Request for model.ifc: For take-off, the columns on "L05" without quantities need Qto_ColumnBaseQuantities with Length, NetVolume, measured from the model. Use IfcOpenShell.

First a look at what the model holds.

```python
import ifcopenshell
import ifcopenshell.util.element
import ifcopenshell.util.unit

model = ifcopenshell.open("model.ifc")
print(model.schema)
for unit_type in ("LENGTHUNIT", "AREAUNIT", "VOLUMEUNIT"):
    print(unit_type, ifcopenshell.util.unit.calculate_unit_scale(model, unit_type))
storey = next(s for s in model.by_type("IfcBuildingStorey") if s.Name == "L05")
columns = [e for e in ifcopenshell.util.element.get_decomposition(storey) if e.is_a("IfcColumn")]
for e in sorted(columns, key=lambda e: e.id()):
    print(e.id(), e.is_a(), e.Name, list(ifcopenshell.util.element.get_psets(e, qtos_only=True)), sep=" | ")
```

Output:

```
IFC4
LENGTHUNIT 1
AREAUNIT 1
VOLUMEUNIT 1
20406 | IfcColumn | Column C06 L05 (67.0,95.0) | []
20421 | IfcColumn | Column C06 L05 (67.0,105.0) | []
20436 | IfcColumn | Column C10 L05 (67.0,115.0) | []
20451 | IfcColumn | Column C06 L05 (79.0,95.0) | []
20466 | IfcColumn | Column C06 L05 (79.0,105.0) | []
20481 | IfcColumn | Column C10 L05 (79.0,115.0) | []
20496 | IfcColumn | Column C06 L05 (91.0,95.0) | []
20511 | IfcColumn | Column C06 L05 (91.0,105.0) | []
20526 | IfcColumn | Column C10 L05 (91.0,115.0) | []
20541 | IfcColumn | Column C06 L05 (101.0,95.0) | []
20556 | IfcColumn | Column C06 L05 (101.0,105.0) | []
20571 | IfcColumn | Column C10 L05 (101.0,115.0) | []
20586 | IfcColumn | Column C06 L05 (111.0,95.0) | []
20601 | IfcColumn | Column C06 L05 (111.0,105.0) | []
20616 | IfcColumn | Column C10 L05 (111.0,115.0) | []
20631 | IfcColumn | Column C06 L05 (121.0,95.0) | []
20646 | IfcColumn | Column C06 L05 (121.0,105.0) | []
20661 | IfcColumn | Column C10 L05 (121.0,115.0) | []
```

```python
import ifcopenshell
import ifcopenshell.api.pset
import ifcopenshell.geom
import ifcopenshell.util.element
import ifcopenshell.util.shape
import ifcopenshell.util.unit

model = ifcopenshell.open("model.ifc")
unit_scale = ifcopenshell.util.unit.calculate_unit_scale(model)
volume_scale = ifcopenshell.util.unit.calculate_unit_scale(model, "VOLUMEUNIT")
settings = ifcopenshell.geom.settings()

storey = next(s for s in model.by_type("IfcBuildingStorey") if s.Name == "L05")
columns = [e for e in ifcopenshell.util.element.get_decomposition(storey) if e.is_a("IfcColumn")]

for e in sorted(columns, key=lambda e: e.id()):
    if ifcopenshell.util.element.get_psets(e, qtos_only=True, should_inherit=False):
        continue
    # Geometry comes back in metres, in the element's own axes.
    shape = ifcopenshell.geom.create_shape(settings, e)
    values = {
        "Length": ifcopenshell.util.shape.get_z(shape.geometry) / unit_scale,
        "NetVolume": ifcopenshell.util.shape.get_volume(shape.geometry) / volume_scale,
    }
    qto = ifcopenshell.api.pset.add_qto(model, product=e, name="Qto_ColumnBaseQuantities")
    ifcopenshell.api.pset.edit_qto(model, qto=qto, properties=values)
    print(e.id(), {k: round(v, 3) for k, v in values.items()})

model.write("model_v2.ifc")
```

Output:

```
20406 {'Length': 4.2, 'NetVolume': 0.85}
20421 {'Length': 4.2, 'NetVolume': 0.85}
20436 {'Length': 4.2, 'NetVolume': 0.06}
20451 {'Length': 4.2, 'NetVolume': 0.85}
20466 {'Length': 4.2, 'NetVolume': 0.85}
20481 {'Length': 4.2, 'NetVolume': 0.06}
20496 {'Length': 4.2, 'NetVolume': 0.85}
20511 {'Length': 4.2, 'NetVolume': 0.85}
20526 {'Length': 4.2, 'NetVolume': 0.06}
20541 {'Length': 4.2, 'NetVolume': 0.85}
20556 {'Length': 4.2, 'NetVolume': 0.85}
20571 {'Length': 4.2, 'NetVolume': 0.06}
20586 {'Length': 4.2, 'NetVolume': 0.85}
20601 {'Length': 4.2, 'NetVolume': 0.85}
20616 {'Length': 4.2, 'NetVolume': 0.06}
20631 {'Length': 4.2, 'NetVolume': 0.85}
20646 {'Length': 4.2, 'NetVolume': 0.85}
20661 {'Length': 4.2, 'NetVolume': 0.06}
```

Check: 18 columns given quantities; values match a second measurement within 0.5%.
